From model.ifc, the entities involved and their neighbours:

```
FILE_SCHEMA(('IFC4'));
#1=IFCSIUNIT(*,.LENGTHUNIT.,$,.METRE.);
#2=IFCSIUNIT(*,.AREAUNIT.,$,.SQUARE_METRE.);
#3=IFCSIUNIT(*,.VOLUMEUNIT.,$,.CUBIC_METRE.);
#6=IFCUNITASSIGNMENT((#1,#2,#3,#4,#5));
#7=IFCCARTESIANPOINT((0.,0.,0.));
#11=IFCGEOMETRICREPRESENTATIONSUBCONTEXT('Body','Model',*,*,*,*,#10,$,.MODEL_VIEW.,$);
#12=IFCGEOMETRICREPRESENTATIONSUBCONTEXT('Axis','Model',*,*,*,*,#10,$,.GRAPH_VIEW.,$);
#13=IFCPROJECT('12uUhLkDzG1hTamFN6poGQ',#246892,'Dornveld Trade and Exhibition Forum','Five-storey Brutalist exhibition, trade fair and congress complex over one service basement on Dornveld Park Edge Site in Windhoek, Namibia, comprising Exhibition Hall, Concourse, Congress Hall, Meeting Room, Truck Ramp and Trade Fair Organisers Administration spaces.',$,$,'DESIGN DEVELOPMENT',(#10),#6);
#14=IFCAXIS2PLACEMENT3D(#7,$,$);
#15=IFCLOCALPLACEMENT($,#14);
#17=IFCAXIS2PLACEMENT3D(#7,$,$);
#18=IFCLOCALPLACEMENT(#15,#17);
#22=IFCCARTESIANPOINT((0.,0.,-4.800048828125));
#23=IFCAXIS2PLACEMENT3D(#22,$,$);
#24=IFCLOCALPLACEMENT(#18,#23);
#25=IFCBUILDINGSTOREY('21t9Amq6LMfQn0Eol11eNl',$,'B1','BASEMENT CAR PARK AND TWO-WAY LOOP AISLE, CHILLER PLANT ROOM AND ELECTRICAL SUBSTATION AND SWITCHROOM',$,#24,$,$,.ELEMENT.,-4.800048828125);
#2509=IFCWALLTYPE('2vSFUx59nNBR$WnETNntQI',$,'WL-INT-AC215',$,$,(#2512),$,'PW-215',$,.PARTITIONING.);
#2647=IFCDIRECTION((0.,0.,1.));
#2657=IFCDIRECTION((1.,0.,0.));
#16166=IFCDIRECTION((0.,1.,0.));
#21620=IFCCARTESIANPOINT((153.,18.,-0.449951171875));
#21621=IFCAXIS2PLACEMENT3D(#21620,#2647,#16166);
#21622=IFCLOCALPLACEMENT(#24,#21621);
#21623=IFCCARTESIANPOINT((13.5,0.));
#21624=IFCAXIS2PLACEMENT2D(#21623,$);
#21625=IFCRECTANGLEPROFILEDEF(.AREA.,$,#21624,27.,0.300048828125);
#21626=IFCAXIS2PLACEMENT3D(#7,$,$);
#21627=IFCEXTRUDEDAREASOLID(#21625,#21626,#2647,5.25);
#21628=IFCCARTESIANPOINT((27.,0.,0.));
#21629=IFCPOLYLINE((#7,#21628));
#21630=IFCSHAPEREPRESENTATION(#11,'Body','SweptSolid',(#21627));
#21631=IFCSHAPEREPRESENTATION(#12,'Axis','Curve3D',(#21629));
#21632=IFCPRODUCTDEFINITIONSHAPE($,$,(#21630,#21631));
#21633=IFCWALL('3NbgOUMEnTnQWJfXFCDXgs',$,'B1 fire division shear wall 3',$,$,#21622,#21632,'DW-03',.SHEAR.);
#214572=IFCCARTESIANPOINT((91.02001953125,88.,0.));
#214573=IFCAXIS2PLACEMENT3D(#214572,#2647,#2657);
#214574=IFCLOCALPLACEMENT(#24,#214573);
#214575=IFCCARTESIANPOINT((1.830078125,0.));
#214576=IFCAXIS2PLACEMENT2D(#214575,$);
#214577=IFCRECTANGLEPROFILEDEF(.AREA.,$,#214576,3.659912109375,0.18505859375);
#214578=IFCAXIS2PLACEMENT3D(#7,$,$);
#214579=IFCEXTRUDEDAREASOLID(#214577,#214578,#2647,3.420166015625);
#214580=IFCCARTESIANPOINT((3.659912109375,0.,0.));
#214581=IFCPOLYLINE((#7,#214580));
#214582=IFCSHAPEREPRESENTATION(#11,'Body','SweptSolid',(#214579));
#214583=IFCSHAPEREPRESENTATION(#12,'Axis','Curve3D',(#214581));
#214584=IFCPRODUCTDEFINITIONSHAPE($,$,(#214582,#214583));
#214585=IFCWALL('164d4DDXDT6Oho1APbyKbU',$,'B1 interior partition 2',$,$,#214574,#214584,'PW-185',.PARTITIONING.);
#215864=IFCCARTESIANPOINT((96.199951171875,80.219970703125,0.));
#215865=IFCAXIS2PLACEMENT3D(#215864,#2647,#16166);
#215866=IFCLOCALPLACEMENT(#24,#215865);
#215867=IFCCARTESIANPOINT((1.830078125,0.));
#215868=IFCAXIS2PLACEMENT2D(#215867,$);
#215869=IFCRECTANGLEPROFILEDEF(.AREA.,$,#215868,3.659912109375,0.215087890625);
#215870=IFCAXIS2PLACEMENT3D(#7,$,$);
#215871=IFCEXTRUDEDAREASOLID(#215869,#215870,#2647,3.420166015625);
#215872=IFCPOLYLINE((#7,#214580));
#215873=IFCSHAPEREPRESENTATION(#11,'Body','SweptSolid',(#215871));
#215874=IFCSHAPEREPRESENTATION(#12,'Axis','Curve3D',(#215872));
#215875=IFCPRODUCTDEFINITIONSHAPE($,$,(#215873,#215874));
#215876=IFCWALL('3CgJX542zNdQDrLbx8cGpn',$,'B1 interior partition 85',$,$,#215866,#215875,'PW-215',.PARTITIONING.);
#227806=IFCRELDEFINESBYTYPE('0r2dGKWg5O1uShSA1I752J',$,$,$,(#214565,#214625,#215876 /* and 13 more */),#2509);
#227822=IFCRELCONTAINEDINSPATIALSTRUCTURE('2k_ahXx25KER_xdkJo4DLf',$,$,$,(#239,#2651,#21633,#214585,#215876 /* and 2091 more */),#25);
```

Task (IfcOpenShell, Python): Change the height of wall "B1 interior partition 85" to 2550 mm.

```python
import ifcopenshell
import ifcopenshell.geom
import ifcopenshell.util.representation
import ifcopenshell.util.shape
import ifcopenshell.util.unit

model = ifcopenshell.open("model.ifc")
unit_scale = ifcopenshell.util.unit.calculate_unit_scale(model)
settings = ifcopenshell.geom.settings()


def volume(element):
    """Net volume in cubic metres, openings subtracted."""
    shape = ifcopenshell.geom.create_shape(settings, element)
    return ifcopenshell.util.shape.get_volume(shape.geometry)


wall = model.by_id(215876)
before = volume(wall)

body = ifcopenshell.util.representation.get_representation(wall, "Model", "Body")
solid = body.Items[0]
old_height = solid.Depth
solid.Depth = 2.55 / unit_scale
after = volume(wall)

print(f"height {old_height:g} -> {solid.Depth:g}, volume {before:.3f} -> {after:.3f} m3")

model.write("model_v2.ifc")
```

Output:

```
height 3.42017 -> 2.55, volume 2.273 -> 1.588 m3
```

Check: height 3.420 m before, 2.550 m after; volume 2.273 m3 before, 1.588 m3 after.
